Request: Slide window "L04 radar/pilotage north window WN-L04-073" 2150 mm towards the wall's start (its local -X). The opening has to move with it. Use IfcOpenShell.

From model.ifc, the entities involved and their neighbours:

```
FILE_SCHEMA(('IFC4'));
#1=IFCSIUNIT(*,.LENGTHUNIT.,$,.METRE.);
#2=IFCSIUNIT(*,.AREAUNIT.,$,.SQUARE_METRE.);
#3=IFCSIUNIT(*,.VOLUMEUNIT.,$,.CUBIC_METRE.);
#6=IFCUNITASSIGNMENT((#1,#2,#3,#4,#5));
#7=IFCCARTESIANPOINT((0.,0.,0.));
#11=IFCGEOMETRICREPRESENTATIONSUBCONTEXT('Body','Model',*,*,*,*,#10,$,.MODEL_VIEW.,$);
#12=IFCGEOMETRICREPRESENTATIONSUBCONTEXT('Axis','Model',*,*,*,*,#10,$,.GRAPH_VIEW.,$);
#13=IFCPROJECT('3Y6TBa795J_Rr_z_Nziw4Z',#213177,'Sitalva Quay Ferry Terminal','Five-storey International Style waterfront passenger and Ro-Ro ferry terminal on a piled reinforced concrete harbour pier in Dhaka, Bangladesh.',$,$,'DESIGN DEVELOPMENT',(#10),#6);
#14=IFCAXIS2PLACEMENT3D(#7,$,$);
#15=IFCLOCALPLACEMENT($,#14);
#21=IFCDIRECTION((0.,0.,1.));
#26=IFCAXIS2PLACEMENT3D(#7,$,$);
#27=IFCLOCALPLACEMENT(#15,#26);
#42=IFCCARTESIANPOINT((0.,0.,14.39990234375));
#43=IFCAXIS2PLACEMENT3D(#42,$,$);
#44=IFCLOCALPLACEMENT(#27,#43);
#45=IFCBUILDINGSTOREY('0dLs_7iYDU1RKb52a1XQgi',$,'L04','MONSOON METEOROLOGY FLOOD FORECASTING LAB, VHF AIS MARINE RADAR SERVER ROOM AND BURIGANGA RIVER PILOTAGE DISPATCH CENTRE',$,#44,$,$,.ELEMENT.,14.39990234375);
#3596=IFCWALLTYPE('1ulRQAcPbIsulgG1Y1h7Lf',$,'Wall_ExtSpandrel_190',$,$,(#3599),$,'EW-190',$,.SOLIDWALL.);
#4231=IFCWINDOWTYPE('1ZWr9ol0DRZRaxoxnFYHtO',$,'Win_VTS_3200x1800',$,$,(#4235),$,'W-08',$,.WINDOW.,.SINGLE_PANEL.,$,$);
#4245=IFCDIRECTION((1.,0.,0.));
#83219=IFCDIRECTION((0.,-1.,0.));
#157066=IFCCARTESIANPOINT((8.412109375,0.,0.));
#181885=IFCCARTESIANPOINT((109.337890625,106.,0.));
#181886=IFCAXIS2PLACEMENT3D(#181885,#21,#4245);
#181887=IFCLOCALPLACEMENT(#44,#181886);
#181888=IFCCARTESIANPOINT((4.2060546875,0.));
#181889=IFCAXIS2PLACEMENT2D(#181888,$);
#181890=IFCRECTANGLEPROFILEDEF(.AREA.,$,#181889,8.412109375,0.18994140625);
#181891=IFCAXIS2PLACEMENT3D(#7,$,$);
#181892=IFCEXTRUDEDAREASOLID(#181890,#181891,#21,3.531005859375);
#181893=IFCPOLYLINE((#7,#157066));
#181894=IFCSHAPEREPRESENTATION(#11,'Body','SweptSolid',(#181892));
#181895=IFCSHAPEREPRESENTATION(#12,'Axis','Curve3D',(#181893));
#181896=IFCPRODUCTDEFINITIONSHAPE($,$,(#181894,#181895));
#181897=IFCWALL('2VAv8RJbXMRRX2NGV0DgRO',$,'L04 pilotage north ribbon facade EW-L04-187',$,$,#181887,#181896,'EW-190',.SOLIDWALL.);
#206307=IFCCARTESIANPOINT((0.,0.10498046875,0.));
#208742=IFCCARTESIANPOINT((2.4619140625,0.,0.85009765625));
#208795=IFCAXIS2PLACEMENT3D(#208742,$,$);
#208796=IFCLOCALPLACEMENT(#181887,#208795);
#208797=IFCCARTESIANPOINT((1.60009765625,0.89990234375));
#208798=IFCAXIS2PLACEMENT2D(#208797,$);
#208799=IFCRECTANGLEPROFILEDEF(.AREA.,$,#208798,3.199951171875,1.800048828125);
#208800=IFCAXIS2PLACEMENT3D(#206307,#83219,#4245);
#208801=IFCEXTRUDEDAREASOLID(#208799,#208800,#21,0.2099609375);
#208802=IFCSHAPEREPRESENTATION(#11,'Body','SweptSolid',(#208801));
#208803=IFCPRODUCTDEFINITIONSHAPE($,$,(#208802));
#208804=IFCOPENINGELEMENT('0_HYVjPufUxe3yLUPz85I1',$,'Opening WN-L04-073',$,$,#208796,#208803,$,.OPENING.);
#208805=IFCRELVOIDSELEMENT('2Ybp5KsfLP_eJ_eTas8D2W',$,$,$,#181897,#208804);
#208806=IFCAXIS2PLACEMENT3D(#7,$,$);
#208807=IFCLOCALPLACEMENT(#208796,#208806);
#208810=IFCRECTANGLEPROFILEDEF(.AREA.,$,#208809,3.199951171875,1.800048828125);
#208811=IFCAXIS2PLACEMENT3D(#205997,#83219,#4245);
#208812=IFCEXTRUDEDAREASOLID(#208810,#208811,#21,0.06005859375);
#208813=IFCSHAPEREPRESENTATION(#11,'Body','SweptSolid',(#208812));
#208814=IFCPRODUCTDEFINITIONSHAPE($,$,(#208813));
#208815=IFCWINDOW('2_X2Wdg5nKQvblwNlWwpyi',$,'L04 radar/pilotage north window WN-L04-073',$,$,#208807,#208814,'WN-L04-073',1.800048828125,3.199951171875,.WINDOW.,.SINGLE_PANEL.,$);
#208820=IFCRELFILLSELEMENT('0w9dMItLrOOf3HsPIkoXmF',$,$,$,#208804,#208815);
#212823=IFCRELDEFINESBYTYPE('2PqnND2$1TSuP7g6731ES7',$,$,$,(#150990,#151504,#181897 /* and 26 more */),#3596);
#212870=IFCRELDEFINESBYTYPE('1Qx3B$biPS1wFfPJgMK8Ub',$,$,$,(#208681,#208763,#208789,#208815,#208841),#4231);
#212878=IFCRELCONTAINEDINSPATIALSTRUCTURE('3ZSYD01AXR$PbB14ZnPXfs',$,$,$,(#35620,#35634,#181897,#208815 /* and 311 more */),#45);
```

```python
import ifcopenshell
import ifcopenshell.api.geometry
import ifcopenshell.util.placement
import ifcopenshell.util.unit

model = ifcopenshell.open("model.ifc")
unit_scale = ifcopenshell.util.unit.calculate_unit_scale(model)

window = model.by_guid("2_X2Wdg5nKQvblwNlWwpyi")
opening = window.FillsVoids[0].RelatingOpeningElement
wall = opening.VoidsElements[0].RelatingBuildingElement

wall_matrix = ifcopenshell.util.placement.get_local_placement(wall.ObjectPlacement)
shift = wall_matrix[:3, 0] * -2.15 / unit_scale
before = ifcopenshell.util.placement.get_local_placement(window.ObjectPlacement)[:3, 3].copy()

# The window is placed relative to its opening, so it follows when the opening moves.
matrix = ifcopenshell.util.placement.get_local_placement(opening.ObjectPlacement)
matrix[:3, 3] += shift
ifcopenshell.api.geometry.edit_object_placement(
    model, product=opening, matrix=matrix, is_si=False, should_transform_children=True
)

after = ifcopenshell.util.placement.get_local_placement(window.ObjectPlacement)[:3, 3]
print("window moved by", (after - before).round(3) + 0.0)

model.write("model_edited.ifc")
```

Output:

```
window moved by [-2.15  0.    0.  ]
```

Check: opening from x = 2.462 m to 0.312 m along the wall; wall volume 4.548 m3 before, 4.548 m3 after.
